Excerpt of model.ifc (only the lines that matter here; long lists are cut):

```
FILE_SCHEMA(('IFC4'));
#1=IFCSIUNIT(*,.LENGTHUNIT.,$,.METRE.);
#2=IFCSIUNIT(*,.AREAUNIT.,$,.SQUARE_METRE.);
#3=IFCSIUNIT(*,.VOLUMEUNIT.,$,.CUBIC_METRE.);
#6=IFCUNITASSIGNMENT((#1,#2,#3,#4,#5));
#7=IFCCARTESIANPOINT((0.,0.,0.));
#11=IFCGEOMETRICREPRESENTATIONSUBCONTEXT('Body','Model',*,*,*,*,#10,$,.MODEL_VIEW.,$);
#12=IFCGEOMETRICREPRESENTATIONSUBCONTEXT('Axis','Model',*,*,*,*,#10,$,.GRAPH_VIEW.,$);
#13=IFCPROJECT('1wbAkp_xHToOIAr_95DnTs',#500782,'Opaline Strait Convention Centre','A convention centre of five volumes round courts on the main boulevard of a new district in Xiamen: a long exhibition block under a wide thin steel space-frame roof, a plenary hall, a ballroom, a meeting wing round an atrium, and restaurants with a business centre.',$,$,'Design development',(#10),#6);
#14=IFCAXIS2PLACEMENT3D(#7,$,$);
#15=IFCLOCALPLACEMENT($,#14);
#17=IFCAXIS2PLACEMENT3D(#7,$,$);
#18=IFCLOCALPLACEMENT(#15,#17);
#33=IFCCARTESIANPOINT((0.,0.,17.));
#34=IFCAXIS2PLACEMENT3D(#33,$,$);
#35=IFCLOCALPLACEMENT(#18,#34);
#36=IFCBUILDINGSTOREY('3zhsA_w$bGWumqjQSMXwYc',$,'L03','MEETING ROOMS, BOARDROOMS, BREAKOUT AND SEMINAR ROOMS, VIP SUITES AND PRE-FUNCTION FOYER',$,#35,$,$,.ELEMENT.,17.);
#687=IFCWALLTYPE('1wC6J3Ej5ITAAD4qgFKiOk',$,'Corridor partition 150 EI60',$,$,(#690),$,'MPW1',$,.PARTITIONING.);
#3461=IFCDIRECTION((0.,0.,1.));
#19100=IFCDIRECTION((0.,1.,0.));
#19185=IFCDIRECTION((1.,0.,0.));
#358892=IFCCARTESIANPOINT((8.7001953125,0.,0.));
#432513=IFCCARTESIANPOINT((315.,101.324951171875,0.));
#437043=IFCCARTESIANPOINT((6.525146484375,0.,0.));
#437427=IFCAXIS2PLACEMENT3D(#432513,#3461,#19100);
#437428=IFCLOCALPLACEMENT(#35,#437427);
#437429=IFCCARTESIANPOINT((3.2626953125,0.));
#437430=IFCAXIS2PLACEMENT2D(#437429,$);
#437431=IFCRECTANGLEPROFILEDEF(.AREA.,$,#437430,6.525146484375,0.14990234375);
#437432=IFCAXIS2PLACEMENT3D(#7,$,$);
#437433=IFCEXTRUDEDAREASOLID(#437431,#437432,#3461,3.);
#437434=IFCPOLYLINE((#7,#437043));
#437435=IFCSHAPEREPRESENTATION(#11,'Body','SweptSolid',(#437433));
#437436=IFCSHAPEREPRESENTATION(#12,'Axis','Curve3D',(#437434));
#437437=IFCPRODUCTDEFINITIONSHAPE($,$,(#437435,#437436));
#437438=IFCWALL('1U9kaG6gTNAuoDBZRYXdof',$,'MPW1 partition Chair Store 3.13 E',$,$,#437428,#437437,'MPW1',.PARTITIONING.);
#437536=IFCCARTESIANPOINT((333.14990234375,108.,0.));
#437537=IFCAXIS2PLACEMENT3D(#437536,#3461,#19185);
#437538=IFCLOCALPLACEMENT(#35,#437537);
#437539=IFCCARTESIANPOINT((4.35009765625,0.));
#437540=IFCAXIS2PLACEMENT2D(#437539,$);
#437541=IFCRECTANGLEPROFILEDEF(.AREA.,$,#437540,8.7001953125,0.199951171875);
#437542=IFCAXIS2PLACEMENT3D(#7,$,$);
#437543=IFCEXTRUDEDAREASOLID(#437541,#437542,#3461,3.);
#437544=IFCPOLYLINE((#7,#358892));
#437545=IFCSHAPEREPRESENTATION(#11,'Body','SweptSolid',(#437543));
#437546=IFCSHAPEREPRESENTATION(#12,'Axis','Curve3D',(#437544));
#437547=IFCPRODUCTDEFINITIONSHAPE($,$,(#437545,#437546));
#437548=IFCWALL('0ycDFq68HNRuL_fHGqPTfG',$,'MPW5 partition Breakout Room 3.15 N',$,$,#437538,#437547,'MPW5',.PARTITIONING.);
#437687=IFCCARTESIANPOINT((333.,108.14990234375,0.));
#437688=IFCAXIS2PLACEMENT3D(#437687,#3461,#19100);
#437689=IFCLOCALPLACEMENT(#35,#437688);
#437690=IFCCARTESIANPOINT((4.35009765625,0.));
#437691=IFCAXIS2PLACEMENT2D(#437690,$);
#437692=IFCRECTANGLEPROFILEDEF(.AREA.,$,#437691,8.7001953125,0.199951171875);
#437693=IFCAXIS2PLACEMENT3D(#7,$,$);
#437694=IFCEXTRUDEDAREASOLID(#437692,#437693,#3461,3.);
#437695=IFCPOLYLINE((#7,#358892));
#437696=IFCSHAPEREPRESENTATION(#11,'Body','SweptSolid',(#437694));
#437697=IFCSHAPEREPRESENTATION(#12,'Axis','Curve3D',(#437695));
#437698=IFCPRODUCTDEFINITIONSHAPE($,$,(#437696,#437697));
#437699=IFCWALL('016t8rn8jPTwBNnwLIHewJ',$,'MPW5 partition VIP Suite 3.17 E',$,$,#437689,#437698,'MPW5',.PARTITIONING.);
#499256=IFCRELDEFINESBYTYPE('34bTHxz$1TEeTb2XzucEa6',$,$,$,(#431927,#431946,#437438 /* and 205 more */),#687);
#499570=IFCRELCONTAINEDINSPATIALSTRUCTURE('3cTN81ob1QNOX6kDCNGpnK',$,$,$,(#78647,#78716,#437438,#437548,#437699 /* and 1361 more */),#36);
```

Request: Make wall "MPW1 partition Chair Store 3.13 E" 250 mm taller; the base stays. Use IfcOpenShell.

```python
import ifcopenshell
import ifcopenshell.geom
import ifcopenshell.util.representation
import ifcopenshell.util.shape

model = ifcopenshell.open("model.ifc")
settings = ifcopenshell.geom.settings()


def volume(element):
    """Net volume in cubic metres, openings subtracted."""
    shape = ifcopenshell.geom.create_shape(settings, element)
    return ifcopenshell.util.shape.get_volume(shape.geometry)


wall = model.by_guid("1U9kaG6gTNAuoDBZRYXdof")
before = volume(wall)

body = ifcopenshell.util.representation.get_representation(wall, "Model", "Body")
solid = body.Items[0]
old_height = solid.Depth
solid.Depth += 0.25
after = volume(wall)

print(f"height {old_height:g} -> {solid.Depth:g}, volume {before:.3f} -> {after:.3f} m3")

model.write("model-out.ifc")
```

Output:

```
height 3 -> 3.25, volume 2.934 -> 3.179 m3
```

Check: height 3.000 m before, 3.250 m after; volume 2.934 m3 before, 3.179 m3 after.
